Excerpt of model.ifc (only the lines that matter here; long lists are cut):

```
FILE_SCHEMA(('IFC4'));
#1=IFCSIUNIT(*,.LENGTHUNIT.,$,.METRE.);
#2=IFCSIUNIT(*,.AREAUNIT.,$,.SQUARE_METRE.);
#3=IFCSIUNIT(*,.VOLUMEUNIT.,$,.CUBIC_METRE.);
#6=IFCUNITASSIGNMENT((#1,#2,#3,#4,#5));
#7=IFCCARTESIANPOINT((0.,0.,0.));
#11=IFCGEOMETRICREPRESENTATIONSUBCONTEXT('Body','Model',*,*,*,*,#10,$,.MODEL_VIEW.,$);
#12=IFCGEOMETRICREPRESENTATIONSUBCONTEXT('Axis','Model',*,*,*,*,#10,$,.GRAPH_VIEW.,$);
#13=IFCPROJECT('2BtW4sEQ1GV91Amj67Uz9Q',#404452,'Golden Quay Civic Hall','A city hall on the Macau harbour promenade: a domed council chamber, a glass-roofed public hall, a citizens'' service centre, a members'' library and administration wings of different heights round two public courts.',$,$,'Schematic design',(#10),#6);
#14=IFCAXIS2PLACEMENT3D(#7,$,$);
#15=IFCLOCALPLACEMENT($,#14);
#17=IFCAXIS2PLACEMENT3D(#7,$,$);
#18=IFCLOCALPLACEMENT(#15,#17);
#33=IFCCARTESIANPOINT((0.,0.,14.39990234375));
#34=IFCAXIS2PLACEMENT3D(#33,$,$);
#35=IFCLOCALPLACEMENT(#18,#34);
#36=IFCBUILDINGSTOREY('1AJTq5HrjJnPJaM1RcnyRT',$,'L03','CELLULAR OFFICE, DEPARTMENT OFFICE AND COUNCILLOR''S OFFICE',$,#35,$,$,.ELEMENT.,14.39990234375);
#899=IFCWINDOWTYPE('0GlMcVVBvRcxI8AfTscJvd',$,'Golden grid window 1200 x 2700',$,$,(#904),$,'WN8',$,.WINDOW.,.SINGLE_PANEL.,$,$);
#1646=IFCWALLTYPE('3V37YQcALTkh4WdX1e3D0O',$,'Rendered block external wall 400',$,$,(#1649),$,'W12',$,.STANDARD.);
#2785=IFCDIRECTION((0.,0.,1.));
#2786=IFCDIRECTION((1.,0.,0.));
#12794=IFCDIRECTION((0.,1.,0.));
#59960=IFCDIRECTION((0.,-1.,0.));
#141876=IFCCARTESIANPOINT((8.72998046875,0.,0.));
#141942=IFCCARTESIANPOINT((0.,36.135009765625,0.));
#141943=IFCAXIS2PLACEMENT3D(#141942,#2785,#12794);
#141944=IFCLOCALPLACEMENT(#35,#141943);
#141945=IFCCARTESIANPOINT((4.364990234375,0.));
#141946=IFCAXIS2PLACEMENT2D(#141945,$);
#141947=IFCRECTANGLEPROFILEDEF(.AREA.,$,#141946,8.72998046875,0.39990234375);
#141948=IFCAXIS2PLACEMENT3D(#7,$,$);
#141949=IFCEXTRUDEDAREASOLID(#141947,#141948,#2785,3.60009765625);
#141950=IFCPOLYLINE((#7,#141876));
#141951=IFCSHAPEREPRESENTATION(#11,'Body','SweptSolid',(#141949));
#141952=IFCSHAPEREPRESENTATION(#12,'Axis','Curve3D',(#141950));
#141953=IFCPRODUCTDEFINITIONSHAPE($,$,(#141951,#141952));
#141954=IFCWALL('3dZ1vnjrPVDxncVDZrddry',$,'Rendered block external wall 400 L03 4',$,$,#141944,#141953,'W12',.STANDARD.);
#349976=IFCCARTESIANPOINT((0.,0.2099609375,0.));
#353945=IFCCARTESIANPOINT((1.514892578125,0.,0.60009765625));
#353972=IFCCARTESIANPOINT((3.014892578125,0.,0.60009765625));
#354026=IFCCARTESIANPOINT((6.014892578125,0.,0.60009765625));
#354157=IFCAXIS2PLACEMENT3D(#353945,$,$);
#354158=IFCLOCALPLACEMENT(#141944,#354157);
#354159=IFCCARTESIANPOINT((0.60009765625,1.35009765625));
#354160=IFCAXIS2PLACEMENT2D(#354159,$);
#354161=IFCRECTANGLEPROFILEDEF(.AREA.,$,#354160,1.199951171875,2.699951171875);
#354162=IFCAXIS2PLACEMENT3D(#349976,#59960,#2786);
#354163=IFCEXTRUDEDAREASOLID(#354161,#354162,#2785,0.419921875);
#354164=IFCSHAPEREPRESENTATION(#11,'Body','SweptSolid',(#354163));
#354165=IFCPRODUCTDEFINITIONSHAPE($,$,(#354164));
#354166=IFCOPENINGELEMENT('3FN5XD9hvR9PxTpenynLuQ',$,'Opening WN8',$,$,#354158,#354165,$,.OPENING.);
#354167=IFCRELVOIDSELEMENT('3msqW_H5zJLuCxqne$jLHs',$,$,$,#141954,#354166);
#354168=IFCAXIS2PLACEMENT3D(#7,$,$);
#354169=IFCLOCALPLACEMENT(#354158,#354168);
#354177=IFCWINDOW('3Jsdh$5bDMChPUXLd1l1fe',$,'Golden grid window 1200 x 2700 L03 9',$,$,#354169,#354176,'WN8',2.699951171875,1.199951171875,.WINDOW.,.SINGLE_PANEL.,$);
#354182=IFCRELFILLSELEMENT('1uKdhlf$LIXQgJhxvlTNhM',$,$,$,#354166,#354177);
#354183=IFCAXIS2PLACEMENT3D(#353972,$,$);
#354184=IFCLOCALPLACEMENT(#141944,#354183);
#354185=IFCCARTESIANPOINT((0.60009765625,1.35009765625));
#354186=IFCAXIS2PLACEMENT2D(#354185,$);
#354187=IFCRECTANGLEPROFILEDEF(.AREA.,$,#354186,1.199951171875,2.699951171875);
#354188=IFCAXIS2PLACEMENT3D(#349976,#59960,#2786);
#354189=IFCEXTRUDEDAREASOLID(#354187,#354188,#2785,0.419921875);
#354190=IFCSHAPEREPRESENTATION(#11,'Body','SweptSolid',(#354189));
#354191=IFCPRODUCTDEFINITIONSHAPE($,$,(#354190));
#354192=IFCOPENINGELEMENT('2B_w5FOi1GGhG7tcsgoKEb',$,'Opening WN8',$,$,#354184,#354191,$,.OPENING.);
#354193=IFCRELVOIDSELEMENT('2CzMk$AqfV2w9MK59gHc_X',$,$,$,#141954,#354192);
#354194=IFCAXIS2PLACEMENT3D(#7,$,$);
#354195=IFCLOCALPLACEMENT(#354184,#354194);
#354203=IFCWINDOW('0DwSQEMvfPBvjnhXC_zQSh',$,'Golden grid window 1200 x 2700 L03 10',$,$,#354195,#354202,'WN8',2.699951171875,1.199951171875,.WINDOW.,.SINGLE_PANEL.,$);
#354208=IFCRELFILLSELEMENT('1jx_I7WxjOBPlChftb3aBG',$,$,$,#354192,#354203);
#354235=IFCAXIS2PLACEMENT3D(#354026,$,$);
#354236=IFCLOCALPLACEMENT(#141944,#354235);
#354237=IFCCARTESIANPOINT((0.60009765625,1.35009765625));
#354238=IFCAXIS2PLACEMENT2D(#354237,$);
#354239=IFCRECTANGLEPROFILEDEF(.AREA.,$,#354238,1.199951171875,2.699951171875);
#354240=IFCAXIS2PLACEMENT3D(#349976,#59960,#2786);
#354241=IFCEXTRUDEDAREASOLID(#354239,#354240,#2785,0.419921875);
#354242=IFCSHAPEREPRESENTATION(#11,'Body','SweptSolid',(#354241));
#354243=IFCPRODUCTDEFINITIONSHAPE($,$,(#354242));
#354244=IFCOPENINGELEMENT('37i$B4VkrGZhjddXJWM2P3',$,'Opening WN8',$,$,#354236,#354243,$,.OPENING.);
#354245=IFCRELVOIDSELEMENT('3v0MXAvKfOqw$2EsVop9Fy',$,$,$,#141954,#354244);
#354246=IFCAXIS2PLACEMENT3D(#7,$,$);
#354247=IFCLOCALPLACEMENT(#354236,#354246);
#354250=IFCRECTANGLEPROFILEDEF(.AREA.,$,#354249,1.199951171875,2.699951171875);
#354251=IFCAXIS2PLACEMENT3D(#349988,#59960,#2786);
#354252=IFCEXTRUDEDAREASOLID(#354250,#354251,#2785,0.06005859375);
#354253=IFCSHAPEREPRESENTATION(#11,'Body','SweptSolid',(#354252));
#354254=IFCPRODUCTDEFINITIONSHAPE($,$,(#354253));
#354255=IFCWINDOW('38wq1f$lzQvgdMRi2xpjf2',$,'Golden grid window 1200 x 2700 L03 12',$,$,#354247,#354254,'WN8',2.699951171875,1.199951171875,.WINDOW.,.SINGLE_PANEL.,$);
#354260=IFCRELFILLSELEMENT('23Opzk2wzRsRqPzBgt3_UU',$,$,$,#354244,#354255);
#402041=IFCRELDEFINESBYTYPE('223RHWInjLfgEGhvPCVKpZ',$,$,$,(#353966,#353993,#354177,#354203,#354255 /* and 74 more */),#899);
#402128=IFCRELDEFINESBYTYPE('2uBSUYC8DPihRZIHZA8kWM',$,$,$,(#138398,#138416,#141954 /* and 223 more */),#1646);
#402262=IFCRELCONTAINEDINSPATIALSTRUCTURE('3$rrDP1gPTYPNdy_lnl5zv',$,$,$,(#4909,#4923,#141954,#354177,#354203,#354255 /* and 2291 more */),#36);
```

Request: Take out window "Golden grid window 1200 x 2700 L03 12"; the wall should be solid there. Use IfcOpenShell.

```python
import ifcopenshell
import ifcopenshell.api.feature
import ifcopenshell.api.root
import ifcopenshell.geom
import ifcopenshell.util.shape

model = ifcopenshell.open("model.ifc")
settings = ifcopenshell.geom.settings()


def volume(element):
    """Net volume in cubic metres, openings subtracted."""
    shape = ifcopenshell.geom.create_shape(settings, element)
    return ifcopenshell.util.shape.get_volume(shape.geometry)


window = model.by_guid("38wq1f$lzQvgdMRi2xpjf2")
opening = window.FillsVoids[0].RelatingOpeningElement
wall = opening.VoidsElements[0].RelatingBuildingElement
before = volume(wall)

ifcopenshell.api.root.remove_product(model, product=window)
ifcopenshell.api.feature.remove_feature(model, feature=opening)

after = volume(wall)

print(f"wall volume {before:.3f} -> {after:.3f} m3")

model.write("model-out.ifc")
```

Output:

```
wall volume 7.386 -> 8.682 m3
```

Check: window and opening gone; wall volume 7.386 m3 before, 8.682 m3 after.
